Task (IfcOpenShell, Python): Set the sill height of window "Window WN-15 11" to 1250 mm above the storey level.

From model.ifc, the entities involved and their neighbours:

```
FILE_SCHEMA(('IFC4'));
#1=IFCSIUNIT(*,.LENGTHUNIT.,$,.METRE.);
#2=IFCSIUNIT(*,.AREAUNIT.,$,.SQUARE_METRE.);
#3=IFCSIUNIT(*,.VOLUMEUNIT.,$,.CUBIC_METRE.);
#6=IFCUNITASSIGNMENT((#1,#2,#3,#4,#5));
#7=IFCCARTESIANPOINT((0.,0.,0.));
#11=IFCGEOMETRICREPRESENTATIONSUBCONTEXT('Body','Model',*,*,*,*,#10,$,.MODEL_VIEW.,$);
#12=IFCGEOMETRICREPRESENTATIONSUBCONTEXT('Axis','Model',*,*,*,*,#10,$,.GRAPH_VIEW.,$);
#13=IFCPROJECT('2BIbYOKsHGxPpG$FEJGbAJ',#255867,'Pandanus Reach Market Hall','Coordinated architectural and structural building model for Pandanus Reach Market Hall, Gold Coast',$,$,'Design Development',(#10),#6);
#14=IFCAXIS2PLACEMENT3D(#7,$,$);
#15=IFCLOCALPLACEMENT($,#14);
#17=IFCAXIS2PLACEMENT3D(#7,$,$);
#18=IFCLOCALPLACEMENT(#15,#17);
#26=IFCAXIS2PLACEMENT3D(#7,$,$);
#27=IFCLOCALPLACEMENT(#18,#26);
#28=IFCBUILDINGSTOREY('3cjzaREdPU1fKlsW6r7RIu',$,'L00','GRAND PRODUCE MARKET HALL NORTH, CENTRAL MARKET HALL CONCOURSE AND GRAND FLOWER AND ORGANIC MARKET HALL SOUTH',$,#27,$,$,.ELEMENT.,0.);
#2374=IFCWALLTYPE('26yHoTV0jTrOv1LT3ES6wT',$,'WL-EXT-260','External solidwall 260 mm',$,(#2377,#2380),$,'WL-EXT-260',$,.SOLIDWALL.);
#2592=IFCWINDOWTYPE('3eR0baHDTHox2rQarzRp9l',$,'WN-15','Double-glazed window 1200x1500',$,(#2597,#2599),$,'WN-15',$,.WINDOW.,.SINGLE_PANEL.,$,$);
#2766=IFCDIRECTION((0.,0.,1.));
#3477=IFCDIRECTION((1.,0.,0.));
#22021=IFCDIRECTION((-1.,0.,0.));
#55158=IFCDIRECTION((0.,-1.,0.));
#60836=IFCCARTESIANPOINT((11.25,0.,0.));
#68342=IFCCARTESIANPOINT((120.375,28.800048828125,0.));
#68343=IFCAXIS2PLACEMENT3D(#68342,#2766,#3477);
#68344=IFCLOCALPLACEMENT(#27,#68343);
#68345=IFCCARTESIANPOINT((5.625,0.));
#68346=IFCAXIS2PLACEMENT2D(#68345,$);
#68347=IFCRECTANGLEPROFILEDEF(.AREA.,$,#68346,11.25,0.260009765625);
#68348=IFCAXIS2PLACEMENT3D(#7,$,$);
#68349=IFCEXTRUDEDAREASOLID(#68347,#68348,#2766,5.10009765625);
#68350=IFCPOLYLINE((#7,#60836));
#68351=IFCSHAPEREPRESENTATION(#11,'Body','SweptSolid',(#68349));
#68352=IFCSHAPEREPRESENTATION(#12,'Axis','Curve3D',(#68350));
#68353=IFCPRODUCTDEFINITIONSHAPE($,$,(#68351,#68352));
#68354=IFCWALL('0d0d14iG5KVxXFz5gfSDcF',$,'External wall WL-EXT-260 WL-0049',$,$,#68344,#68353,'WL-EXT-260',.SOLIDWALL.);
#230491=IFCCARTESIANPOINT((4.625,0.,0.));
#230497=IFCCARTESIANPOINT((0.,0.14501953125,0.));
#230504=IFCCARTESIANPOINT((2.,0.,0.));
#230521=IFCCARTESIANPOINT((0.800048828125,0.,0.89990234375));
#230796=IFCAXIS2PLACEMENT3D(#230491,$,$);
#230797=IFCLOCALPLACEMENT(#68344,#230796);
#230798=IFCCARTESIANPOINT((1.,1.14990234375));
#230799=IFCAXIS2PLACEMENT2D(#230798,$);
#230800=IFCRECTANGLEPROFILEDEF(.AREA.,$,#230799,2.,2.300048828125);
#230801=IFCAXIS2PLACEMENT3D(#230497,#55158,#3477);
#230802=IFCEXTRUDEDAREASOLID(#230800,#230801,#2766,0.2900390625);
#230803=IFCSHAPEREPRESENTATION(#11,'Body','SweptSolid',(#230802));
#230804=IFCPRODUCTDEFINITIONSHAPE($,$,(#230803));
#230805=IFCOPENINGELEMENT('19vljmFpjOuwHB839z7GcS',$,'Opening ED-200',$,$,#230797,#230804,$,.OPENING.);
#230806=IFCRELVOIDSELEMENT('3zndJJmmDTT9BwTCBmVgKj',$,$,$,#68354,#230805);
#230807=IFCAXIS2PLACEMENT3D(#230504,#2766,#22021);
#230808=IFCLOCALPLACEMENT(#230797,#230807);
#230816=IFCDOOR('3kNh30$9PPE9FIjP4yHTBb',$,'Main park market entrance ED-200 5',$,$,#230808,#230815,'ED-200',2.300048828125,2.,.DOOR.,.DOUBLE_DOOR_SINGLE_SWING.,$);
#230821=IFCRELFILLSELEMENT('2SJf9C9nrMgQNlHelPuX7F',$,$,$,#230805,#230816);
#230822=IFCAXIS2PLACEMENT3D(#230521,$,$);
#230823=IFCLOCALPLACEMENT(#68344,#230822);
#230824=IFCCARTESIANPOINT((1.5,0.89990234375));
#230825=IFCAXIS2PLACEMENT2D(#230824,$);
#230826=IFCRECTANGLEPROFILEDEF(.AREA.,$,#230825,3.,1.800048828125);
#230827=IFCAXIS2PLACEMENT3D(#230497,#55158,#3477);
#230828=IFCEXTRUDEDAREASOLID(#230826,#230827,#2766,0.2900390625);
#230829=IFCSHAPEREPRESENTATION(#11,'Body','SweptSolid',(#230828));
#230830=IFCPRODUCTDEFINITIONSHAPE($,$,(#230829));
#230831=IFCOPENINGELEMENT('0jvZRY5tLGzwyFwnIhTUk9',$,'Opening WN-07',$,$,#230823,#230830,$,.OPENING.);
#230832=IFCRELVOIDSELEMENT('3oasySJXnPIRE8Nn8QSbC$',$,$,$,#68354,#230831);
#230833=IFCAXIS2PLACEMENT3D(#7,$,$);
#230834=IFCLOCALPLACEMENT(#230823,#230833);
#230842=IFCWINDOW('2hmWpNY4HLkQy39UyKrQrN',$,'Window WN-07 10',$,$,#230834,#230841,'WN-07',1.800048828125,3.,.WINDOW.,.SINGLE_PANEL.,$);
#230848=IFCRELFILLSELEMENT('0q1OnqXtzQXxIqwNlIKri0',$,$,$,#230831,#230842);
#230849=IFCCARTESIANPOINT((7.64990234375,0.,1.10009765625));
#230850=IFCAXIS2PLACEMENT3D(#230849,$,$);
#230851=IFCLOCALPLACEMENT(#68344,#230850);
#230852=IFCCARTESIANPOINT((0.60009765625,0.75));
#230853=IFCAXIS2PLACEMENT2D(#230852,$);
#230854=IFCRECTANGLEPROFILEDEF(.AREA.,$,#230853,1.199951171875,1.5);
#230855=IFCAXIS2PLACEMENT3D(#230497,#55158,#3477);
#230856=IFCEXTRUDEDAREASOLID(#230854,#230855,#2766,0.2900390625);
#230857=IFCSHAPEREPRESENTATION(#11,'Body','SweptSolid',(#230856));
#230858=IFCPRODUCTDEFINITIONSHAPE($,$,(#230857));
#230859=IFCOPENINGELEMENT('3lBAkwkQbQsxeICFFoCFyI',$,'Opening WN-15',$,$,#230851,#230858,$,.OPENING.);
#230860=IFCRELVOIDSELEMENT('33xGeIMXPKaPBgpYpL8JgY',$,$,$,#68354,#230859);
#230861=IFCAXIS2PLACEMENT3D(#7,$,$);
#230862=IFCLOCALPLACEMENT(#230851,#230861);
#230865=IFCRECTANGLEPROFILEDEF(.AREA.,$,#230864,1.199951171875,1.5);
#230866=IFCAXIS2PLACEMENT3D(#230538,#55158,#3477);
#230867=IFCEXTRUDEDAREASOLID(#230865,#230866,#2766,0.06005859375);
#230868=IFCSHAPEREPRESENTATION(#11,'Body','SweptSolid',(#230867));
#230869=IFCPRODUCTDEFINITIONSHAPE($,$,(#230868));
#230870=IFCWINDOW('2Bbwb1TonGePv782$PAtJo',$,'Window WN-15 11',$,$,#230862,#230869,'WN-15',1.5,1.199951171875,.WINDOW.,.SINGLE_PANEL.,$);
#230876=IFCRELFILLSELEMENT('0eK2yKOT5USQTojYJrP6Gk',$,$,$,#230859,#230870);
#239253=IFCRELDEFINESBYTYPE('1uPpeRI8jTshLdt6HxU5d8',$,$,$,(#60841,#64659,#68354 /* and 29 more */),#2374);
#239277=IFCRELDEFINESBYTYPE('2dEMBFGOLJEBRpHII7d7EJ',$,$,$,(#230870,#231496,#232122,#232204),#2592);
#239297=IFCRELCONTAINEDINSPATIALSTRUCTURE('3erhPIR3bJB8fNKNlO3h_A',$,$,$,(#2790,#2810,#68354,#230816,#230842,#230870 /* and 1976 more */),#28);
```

```python
import numpy as np
import ifcopenshell
import ifcopenshell.api.geometry
import ifcopenshell.geom
import ifcopenshell.util.element
import ifcopenshell.util.placement
import ifcopenshell.util.shape
import ifcopenshell.util.unit

model = ifcopenshell.open("model.ifc")
unit_scale = ifcopenshell.util.unit.calculate_unit_scale(model)

window = model.by_guid("2Bbwb1TonGePv782$PAtJo")
opening = window.FillsVoids[0].RelatingOpeningElement
storey = ifcopenshell.util.element.get_container(window, ifc_class="IfcBuildingStorey")
level = ifcopenshell.util.placement.get_local_placement(storey.ObjectPlacement)[2, 3]

# The opening's origin need not be at the sill, so measure its lowest point.
shape = ifcopenshell.geom.create_shape(ifcopenshell.geom.settings(), opening)
bottom = ifcopenshell.util.shape.get_shape_bottom_elevation(shape, shape.geometry) / unit_scale
dz = level + 1.25 / unit_scale - bottom

shift = np.array([0.0, 0.0, dz])
# The window is placed relative to its opening, so it follows when the opening moves.
matrix = ifcopenshell.util.placement.get_local_placement(opening.ObjectPlacement)
matrix[:3, 3] += shift
ifcopenshell.api.geometry.edit_object_placement(
    model, product=opening, matrix=matrix, is_si=False, should_transform_children=True
)

print(f"moved by {dz * unit_scale:+.3f} m")

model.write("model_updated.ifc")
```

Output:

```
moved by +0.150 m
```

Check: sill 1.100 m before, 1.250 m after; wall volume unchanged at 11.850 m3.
